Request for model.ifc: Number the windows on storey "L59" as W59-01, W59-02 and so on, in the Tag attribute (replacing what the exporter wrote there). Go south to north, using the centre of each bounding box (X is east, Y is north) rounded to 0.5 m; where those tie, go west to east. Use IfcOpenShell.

First a look at what the model holds.

```python
import ifcopenshell
import ifcopenshell.util.element
import ifcopenshell.util.placement

model = ifcopenshell.open("model.ifc")
print(model.schema)
storey = next(s for s in model.by_type("IfcBuildingStorey") if s.Name == "L59")
windows = [e for e in ifcopenshell.util.element.get_decomposition(storey) if e.is_a("IfcWindow")]
for e in sorted(windows, key=lambda e: e.id()):
    origin = ifcopenshell.util.placement.get_local_placement(e.ObjectPlacement)[:3, 3]
    print(e.id(), e.Tag, e.Name, origin.round(2) + 0.0, sep=" | ")
```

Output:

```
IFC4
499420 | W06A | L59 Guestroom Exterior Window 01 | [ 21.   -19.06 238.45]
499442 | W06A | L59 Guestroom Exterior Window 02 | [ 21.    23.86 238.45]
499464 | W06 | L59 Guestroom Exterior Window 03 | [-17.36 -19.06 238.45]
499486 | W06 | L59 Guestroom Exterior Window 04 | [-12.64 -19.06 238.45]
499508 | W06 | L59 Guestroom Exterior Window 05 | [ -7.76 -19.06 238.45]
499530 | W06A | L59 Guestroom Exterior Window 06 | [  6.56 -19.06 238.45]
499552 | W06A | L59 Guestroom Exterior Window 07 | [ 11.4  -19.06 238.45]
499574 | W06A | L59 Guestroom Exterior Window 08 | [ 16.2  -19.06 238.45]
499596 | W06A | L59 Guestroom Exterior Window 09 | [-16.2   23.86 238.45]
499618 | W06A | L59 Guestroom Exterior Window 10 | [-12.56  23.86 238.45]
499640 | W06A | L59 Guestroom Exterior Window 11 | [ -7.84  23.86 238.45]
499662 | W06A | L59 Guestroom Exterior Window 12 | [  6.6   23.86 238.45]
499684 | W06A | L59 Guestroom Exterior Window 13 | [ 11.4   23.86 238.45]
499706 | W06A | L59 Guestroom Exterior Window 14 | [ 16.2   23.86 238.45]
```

```python
import ifcopenshell
import ifcopenshell.geom
import ifcopenshell.util.element
import ifcopenshell.util.shape

model = ifcopenshell.open("model.ifc")
settings = ifcopenshell.geom.settings()
settings.set("use-world-coords", True)


def centre(element):
    shape = ifcopenshell.geom.create_shape(settings, element)
    return ifcopenshell.util.shape.get_bbox_centroid(shape.geometry)


storey = next(s for s in model.by_type("IfcBuildingStorey") if s.Name == "L59")
windows = [e for e in ifcopenshell.util.element.get_decomposition(storey) if e.is_a("IfcWindow")]

# Insertion points can sit at a corner or the storey origin, so sort by the geometry (in metres).
centres = {e: centre(e) for e in windows}
windows.sort(key=lambda e: (round(centres[e][1] / 0.5), centres[e][0]))

for i, e in enumerate(windows, start=1):
    number = f"W59-{i:02d}"
    e.Tag = number
    print(e.id(), number)

model.write("model_updated.ifc")
```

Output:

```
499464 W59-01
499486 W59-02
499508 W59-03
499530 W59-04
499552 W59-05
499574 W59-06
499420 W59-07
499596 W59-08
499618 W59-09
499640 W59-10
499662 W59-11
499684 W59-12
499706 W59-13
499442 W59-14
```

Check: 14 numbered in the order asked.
